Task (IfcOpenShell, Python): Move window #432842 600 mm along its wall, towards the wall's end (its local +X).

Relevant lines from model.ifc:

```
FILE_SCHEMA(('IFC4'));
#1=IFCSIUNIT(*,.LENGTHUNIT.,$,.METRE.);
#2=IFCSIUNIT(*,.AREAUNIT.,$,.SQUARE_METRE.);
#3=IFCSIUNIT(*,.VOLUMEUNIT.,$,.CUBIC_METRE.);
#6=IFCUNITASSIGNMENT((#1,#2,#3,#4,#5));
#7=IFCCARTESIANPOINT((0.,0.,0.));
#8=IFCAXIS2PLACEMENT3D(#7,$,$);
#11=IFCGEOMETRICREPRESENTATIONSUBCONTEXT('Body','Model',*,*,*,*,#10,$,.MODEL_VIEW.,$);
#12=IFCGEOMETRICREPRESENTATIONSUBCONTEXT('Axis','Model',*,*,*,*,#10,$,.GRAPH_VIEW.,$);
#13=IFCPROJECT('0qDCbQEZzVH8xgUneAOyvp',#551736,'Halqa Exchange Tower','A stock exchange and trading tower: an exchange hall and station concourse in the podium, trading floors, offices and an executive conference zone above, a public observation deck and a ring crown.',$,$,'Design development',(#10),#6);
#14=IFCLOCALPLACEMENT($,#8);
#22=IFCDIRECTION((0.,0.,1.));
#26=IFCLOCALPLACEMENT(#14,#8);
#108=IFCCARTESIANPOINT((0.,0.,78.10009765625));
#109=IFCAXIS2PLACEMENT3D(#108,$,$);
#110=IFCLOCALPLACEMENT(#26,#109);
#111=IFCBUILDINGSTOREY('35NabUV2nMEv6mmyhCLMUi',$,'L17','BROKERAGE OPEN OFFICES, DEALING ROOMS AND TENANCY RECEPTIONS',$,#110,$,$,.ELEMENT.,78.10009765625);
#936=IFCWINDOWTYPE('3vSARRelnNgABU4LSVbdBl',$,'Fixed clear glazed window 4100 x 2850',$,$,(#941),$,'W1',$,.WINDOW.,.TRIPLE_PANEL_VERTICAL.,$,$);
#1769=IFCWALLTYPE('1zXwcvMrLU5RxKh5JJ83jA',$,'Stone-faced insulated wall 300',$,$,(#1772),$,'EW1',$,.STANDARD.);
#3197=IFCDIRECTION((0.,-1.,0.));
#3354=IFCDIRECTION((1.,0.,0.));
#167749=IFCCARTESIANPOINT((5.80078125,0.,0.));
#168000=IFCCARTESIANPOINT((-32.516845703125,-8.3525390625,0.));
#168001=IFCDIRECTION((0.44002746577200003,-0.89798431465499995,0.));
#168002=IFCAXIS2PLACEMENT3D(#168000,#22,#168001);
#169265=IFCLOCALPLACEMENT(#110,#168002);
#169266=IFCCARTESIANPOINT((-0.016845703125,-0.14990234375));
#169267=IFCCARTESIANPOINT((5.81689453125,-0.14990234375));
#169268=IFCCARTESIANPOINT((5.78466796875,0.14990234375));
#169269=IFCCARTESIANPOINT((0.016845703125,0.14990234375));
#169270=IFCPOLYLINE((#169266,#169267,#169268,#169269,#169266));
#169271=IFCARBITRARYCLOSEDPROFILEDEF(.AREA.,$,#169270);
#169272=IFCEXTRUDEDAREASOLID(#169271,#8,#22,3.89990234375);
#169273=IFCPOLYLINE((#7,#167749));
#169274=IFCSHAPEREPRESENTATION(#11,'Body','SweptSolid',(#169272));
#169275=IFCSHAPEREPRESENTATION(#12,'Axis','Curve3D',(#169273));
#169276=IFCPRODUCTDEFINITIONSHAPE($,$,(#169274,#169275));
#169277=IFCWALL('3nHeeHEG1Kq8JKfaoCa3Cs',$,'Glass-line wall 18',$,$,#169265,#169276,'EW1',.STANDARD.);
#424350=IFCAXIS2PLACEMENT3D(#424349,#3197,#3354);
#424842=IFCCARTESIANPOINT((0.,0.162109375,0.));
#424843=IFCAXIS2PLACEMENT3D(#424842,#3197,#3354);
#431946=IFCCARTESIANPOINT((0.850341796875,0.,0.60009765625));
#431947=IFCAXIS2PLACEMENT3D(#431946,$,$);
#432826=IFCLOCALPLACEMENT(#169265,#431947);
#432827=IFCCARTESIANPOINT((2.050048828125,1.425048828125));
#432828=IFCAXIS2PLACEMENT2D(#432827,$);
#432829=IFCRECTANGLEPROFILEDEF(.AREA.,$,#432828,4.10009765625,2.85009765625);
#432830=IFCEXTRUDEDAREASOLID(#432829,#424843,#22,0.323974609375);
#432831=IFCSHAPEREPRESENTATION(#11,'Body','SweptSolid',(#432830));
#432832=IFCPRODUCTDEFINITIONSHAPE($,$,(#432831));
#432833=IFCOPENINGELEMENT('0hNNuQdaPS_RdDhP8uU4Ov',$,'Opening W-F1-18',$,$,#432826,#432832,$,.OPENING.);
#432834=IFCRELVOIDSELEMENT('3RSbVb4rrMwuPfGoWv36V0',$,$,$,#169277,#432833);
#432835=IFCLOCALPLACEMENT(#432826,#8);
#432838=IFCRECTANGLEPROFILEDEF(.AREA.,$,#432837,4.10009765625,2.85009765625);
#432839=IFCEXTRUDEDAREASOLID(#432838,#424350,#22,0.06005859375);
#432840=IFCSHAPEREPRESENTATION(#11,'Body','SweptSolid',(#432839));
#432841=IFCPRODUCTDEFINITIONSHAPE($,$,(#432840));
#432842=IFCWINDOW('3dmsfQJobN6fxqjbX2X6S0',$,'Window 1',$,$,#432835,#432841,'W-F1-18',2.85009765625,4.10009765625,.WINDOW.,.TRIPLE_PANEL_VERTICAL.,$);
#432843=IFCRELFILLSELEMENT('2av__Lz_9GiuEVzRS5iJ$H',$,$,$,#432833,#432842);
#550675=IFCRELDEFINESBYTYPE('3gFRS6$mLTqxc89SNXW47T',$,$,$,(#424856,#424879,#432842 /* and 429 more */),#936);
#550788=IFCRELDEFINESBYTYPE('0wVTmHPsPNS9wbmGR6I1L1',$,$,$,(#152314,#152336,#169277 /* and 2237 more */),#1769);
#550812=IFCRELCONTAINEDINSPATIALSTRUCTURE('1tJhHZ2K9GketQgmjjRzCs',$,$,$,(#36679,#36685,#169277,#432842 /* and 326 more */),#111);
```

```python
import ifcopenshell
import ifcopenshell.api.geometry
import ifcopenshell.util.placement
import ifcopenshell.util.unit

model = ifcopenshell.open("model.ifc")
unit_scale = ifcopenshell.util.unit.calculate_unit_scale(model)

window = model.by_id(432842)
opening = window.FillsVoids[0].RelatingOpeningElement
wall = opening.VoidsElements[0].RelatingBuildingElement

wall_matrix = ifcopenshell.util.placement.get_local_placement(wall.ObjectPlacement)
shift = wall_matrix[:3, 0] * 0.6 / unit_scale
before = ifcopenshell.util.placement.get_local_placement(window.ObjectPlacement)[:3, 3].copy()

# The window is placed relative to its opening, so it follows when the opening moves.
matrix = ifcopenshell.util.placement.get_local_placement(opening.ObjectPlacement)
matrix[:3, 3] += shift
ifcopenshell.api.geometry.edit_object_placement(
    model, product=opening, matrix=matrix, is_si=False, should_transform_children=True
)

after = ifcopenshell.util.placement.get_local_placement(window.ObjectPlacement)[:3, 3]
print("window moved by", (after - before).round(3) + 0.0)

model.write("model-out.ifc")
```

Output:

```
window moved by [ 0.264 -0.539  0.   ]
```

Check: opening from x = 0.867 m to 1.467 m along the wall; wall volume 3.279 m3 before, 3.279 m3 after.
